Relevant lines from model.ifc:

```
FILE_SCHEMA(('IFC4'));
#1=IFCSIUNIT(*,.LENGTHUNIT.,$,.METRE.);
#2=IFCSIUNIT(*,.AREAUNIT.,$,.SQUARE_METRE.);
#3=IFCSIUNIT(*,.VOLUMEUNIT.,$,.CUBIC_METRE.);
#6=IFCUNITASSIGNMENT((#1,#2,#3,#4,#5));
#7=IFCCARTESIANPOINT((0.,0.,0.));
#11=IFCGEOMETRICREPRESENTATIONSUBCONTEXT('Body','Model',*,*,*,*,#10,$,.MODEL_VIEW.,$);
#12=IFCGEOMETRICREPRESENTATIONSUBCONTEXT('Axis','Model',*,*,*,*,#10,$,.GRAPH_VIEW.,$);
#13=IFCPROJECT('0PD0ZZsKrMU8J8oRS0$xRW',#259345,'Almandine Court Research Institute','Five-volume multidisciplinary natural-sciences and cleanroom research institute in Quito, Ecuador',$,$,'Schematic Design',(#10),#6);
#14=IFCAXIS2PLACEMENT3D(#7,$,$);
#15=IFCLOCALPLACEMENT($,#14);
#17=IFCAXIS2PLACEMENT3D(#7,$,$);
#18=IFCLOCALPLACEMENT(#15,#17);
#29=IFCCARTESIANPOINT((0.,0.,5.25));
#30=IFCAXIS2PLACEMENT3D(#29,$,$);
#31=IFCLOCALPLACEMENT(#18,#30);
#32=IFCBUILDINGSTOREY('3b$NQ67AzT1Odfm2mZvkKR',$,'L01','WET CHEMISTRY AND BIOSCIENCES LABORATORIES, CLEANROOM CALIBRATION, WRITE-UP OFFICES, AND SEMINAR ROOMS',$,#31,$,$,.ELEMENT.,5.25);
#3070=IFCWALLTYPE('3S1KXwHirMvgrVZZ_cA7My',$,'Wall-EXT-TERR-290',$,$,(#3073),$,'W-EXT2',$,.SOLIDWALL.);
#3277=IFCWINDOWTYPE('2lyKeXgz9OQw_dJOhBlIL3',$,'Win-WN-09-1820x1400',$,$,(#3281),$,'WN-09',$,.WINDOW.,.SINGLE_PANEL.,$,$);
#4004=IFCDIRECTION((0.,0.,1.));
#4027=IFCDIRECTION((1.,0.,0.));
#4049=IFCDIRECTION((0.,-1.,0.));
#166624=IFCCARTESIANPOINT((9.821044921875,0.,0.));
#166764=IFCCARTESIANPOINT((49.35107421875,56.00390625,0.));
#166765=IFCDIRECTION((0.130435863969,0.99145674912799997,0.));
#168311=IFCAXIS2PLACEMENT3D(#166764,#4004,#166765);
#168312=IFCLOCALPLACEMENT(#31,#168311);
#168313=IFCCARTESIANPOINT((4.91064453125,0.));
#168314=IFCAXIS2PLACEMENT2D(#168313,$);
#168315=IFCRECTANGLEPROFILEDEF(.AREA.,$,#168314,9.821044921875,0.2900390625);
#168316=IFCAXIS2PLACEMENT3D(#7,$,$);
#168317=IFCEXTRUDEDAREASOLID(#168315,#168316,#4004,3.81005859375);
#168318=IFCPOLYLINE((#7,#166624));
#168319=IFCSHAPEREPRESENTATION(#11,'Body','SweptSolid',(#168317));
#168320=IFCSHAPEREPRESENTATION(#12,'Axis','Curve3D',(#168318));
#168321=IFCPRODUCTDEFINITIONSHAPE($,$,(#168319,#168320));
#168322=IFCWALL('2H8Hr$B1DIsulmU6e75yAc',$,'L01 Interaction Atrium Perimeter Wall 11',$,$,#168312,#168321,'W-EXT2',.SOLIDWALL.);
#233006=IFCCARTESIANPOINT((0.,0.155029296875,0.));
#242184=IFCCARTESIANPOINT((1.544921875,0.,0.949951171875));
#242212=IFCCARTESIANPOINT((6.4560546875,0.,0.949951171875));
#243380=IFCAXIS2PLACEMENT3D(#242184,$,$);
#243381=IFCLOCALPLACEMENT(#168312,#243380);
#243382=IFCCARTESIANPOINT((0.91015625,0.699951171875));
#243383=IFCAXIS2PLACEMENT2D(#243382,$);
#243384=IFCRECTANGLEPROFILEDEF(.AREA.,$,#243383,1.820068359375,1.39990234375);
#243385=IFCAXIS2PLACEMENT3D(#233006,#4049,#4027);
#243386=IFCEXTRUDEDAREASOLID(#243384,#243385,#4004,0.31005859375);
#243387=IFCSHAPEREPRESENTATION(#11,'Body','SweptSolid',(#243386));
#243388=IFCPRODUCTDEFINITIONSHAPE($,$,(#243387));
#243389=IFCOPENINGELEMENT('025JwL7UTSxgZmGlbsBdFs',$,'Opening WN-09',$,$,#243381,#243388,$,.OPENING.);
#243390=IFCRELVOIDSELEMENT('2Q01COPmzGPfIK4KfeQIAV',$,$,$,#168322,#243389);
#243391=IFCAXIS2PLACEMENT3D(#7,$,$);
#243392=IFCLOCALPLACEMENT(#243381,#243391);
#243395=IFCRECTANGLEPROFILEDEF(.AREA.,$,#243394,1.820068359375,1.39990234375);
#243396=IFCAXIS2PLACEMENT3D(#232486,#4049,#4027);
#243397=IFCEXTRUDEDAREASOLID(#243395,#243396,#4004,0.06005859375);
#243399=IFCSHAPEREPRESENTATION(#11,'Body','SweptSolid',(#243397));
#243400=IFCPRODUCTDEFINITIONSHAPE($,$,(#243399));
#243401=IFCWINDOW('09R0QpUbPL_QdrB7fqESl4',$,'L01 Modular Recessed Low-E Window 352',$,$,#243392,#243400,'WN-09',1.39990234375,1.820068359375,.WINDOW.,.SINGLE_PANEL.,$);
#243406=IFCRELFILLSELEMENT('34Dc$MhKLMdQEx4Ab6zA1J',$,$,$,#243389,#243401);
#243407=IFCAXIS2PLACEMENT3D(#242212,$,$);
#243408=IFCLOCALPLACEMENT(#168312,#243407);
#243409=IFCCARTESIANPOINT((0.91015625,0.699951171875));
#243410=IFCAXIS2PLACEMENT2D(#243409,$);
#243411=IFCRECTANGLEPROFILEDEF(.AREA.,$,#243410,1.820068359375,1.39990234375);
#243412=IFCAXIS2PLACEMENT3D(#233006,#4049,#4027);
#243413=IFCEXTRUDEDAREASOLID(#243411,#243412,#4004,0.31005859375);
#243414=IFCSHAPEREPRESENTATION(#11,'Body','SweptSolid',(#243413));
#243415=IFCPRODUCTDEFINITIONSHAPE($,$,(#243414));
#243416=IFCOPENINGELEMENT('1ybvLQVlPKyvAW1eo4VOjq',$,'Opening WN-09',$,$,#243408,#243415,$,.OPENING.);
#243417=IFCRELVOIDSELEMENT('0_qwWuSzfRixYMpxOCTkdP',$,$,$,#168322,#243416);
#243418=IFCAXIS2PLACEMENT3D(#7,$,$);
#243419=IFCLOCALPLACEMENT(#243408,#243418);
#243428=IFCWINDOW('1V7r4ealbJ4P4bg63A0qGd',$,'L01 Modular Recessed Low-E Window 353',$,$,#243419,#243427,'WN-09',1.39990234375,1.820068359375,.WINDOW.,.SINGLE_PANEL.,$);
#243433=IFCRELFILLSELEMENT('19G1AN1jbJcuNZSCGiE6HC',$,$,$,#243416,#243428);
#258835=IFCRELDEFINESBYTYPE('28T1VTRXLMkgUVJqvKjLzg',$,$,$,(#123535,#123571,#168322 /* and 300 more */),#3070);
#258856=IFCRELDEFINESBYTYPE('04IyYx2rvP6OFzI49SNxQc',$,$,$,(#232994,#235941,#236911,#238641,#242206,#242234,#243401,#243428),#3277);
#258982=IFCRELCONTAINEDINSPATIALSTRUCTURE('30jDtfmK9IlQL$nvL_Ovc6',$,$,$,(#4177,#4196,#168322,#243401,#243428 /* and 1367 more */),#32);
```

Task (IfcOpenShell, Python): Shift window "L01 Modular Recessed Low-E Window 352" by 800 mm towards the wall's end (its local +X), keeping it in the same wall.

```python
import ifcopenshell
import ifcopenshell.api.geometry
import ifcopenshell.util.placement

model = ifcopenshell.open("model.ifc")

window = model.by_guid("09R0QpUbPL_QdrB7fqESl4")
opening = window.FillsVoids[0].RelatingOpeningElement
wall = opening.VoidsElements[0].RelatingBuildingElement

wall_matrix = ifcopenshell.util.placement.get_local_placement(wall.ObjectPlacement)
shift = wall_matrix[:3, 0] * 0.8
before = ifcopenshell.util.placement.get_local_placement(window.ObjectPlacement)[:3, 3].copy()

# The window is placed relative to its opening, so it follows when the opening moves.
matrix = ifcopenshell.util.placement.get_local_placement(opening.ObjectPlacement)
matrix[:3, 3] += shift
ifcopenshell.api.geometry.edit_object_placement(
    model, product=opening, matrix=matrix, is_si=False, should_transform_children=True
)

after = ifcopenshell.util.placement.get_local_placement(window.ObjectPlacement)[:3, 3]
print("window moved by", (after - before).round(3) + 0.0)

model.write("model_rev.ifc")
```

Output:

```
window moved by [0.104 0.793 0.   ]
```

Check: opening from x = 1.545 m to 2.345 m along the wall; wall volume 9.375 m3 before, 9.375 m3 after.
